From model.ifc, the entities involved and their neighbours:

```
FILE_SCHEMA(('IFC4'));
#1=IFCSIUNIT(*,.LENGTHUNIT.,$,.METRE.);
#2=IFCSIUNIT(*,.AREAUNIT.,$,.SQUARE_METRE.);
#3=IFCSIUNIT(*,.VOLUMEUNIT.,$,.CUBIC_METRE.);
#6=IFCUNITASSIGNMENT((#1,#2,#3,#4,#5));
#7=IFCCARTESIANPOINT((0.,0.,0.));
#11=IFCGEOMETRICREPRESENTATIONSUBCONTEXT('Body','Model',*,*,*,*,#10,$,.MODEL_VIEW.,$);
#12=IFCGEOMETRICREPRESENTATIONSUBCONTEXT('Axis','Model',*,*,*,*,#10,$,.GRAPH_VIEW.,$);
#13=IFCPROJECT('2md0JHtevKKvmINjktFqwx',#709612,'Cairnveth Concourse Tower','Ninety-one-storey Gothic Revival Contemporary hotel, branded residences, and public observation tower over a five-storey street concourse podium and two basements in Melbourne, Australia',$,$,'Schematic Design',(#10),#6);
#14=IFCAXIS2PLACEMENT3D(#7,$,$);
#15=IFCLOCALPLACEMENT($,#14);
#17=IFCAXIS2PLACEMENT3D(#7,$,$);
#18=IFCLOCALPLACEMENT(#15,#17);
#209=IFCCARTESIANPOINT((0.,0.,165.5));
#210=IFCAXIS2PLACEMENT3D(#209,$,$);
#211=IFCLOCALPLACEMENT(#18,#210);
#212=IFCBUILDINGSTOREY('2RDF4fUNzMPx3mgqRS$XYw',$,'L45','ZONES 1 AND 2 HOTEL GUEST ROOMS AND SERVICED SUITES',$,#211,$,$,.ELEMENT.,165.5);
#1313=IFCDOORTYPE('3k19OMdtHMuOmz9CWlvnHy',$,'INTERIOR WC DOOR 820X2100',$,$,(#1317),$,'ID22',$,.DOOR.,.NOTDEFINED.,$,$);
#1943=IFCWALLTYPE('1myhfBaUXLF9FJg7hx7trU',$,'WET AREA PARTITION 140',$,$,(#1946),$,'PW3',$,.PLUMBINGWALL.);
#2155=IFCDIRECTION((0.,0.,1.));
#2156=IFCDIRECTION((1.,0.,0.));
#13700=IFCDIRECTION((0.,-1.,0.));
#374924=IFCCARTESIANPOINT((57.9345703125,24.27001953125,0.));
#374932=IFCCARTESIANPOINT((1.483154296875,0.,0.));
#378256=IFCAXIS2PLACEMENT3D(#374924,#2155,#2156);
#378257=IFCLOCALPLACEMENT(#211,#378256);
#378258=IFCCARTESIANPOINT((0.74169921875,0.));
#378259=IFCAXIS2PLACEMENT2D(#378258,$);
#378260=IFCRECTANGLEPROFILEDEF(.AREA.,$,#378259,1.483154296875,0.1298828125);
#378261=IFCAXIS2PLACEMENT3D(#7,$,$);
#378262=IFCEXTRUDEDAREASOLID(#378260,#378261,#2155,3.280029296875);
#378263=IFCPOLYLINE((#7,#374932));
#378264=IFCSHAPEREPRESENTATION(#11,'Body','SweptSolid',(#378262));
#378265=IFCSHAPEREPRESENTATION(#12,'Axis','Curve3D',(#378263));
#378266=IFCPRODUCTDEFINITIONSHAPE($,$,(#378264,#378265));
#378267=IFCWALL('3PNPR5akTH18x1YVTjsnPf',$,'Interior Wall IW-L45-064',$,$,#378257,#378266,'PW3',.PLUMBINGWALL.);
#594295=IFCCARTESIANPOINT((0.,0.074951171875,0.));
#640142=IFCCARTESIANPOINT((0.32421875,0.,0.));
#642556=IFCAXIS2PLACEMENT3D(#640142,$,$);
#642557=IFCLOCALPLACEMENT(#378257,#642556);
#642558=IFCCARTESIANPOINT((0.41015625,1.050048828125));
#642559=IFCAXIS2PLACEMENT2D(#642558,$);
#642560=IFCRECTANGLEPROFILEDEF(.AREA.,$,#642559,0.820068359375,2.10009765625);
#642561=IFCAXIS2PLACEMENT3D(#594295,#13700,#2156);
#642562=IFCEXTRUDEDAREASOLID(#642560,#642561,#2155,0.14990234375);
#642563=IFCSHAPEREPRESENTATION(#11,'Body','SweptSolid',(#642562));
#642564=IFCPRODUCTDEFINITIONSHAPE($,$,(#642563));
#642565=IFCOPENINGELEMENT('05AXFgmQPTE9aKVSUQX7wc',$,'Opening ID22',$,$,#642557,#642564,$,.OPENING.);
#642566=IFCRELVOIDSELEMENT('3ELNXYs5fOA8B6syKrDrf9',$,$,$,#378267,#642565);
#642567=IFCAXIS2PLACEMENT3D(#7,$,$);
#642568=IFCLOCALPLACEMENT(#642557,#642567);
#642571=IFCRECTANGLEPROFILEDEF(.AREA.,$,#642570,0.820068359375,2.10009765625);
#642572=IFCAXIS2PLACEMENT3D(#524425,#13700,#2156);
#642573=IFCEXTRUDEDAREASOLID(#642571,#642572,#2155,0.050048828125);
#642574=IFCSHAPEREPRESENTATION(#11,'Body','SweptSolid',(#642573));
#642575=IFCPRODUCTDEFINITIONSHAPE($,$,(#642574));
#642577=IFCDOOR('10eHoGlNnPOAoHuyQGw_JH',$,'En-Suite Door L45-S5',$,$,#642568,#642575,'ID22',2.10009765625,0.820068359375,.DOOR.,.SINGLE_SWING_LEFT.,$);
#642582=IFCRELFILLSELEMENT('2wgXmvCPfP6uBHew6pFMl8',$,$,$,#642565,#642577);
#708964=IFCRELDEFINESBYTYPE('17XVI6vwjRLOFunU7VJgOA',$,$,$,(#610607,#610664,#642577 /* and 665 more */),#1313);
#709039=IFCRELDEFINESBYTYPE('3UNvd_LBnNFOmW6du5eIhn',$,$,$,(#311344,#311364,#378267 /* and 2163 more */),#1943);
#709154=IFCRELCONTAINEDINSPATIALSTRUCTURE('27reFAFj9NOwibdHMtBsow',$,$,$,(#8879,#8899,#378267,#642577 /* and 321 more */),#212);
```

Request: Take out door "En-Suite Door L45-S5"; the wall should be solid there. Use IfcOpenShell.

```python
import ifcopenshell
import ifcopenshell.api.feature
import ifcopenshell.api.root
import ifcopenshell.geom
import ifcopenshell.util.shape

model = ifcopenshell.open("model.ifc")
settings = ifcopenshell.geom.settings()


def volume(element):
    """Net volume in cubic metres, openings subtracted."""
    shape = ifcopenshell.geom.create_shape(settings, element)
    return ifcopenshell.util.shape.get_volume(shape.geometry)


door = model.by_guid("10eHoGlNnPOAoHuyQGw_JH")
opening = door.FillsVoids[0].RelatingOpeningElement
wall = opening.VoidsElements[0].RelatingBuildingElement
before = volume(wall)

ifcopenshell.api.root.remove_product(model, product=door)
ifcopenshell.api.feature.remove_feature(model, feature=opening)

after = volume(wall)

print(f"wall volume {before:.3f} -> {after:.3f} m3")

model.write("model_updated.ifc")
```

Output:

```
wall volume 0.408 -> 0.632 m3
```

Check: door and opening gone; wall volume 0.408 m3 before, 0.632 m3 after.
